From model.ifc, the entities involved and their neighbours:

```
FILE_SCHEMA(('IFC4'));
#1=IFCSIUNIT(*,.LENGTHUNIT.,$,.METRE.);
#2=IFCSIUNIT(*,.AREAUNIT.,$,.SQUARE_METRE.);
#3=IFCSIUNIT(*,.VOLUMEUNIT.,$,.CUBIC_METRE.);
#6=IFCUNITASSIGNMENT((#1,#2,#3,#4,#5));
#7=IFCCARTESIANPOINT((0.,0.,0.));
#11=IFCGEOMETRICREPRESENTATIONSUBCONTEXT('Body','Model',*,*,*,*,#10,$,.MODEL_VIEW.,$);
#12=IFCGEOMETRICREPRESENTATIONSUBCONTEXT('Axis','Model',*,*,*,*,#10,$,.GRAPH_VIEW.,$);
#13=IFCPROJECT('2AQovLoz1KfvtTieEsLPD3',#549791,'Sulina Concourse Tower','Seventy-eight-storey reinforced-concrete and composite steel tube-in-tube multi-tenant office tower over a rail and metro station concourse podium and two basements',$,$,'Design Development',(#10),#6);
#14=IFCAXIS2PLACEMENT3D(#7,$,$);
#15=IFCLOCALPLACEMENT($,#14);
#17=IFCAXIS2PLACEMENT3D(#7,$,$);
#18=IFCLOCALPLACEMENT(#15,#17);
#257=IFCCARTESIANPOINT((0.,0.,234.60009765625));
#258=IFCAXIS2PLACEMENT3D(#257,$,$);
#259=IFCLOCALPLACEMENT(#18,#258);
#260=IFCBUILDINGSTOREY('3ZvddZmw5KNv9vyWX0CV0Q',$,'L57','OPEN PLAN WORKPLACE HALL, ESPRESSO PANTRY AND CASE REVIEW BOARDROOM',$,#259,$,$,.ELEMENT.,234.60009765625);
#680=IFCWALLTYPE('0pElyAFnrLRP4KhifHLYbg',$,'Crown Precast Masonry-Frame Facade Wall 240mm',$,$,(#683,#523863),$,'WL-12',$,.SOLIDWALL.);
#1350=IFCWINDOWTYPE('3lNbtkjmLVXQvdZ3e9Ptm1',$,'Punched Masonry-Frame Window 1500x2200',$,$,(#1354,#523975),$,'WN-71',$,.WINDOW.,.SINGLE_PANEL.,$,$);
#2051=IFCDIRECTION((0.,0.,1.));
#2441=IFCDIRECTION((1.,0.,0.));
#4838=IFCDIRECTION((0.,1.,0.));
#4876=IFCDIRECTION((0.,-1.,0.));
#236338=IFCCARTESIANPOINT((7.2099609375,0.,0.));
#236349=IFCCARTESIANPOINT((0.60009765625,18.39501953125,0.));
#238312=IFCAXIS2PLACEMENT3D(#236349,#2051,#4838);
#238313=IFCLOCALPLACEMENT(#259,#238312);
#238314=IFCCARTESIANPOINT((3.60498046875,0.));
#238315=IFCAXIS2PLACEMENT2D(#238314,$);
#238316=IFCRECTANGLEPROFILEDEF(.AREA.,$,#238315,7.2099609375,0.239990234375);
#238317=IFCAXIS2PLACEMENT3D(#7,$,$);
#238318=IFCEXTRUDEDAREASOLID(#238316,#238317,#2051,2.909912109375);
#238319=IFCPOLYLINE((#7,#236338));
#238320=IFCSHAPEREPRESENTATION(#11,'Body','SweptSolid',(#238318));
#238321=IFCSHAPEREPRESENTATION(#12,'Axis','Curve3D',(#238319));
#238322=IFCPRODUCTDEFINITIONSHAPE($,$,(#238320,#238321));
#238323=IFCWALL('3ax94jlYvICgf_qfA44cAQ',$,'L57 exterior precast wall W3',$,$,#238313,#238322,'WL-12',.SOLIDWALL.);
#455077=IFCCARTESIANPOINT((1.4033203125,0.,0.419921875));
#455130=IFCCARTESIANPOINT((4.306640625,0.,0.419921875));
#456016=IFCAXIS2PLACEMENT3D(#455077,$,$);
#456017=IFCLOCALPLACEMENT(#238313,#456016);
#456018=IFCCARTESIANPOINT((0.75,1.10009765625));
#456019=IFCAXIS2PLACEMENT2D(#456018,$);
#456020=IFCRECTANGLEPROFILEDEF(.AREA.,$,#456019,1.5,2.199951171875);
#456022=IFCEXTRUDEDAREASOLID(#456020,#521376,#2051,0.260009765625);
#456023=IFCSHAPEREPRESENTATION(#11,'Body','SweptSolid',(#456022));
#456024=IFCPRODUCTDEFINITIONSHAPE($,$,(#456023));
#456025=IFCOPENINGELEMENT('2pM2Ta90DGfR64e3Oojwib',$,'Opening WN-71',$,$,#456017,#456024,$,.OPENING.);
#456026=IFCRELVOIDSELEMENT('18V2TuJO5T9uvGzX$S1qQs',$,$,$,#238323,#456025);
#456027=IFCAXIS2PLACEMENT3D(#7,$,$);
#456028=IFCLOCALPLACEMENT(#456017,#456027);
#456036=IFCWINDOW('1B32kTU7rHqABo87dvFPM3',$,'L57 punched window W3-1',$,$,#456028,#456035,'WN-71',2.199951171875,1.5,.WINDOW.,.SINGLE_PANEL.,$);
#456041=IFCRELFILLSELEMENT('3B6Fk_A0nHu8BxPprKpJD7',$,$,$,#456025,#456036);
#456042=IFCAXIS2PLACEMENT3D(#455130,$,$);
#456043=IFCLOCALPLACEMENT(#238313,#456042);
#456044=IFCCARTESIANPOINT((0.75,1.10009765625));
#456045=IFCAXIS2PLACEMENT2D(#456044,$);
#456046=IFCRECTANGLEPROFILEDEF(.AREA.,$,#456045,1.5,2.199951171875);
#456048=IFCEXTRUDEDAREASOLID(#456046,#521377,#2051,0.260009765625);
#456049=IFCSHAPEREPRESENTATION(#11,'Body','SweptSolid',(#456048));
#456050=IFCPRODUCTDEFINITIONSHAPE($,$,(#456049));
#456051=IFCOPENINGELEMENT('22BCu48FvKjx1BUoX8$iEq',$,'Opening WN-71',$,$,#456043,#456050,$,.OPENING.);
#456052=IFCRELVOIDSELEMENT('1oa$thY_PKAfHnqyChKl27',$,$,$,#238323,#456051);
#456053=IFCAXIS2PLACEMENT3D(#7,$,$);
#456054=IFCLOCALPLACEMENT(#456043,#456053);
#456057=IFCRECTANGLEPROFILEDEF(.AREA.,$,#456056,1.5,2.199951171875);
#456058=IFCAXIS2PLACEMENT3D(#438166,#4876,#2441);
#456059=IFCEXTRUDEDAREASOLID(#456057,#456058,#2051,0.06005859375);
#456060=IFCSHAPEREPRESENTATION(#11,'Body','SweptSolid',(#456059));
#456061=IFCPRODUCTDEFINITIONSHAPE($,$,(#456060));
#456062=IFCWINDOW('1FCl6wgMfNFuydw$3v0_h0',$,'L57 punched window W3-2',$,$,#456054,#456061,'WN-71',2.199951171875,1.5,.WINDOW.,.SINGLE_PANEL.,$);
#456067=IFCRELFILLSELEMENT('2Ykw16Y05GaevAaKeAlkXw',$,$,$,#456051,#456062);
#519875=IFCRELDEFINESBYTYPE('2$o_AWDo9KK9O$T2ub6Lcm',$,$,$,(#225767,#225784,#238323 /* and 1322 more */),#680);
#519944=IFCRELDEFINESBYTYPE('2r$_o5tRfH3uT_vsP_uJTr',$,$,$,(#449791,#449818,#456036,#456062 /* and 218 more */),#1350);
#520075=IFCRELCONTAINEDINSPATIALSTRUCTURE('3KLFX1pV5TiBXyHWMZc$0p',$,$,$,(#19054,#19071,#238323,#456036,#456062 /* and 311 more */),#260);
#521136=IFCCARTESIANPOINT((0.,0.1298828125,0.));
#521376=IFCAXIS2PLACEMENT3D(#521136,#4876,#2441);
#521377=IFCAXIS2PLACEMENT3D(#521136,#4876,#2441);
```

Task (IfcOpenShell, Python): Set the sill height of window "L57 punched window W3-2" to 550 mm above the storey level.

```python
import numpy as np
import ifcopenshell
import ifcopenshell.api.geometry
import ifcopenshell.geom
import ifcopenshell.util.element
import ifcopenshell.util.placement
import ifcopenshell.util.shape
import ifcopenshell.util.unit

model = ifcopenshell.open("model.ifc")
unit_scale = ifcopenshell.util.unit.calculate_unit_scale(model)

window = model.by_id(456062)
opening = window.FillsVoids[0].RelatingOpeningElement
storey = ifcopenshell.util.element.get_container(window, ifc_class="IfcBuildingStorey")
level = ifcopenshell.util.placement.get_local_placement(storey.ObjectPlacement)[2, 3]

# The opening's origin need not be at the sill, so measure its lowest point.
shape = ifcopenshell.geom.create_shape(ifcopenshell.geom.settings(), opening)
bottom = ifcopenshell.util.shape.get_shape_bottom_elevation(shape, shape.geometry) / unit_scale
dz = level + 0.55 - bottom

shift = np.array([0.0, 0.0, dz])
# The window is placed relative to its opening, so it follows when the opening moves.
matrix = ifcopenshell.util.placement.get_local_placement(opening.ObjectPlacement)
matrix[:3, 3] += shift
ifcopenshell.api.geometry.edit_object_placement(
    model, product=opening, matrix=matrix, is_si=False, should_transform_children=True
)

print(f"moved by {dz * unit_scale:+.3f} m")

model.write("model_updated.ifc")
```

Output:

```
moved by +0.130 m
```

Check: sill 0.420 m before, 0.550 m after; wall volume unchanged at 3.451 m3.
